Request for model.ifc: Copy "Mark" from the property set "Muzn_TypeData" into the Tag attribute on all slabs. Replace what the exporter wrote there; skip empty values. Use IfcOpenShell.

First a look at what the model holds.

```python
import ifcopenshell
import ifcopenshell.util.element

model = ifcopenshell.open("model.ifc")
print(model.schema)
slabs = model.by_type("IfcSlab")
print(len(slabs), "slabs")
for e in slabs[:8]:
    source = ifcopenshell.util.element.get_pset(e, "Muzn_TypeData", "Mark")
    target = e.Tag
    print(e.id(), repr(source), repr(target), sep=" | ")
```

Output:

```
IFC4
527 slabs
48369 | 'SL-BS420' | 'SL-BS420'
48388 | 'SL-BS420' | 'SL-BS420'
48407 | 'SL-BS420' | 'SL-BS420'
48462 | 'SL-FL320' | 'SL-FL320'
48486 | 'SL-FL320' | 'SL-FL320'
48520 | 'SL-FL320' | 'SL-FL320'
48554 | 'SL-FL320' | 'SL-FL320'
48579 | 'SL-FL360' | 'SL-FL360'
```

```python
import ifcopenshell
import ifcopenshell.util.element

model = ifcopenshell.open("model.ifc")

count = 0
for e in model.by_type("IfcSlab"):
    value = ifcopenshell.util.element.get_pset(e, "Muzn_TypeData", "Mark")
    current = e.Tag
    if not value or not value.strip() or current == value:
        continue
    e.Tag = value
    count += 1

print(count, "slabs updated")

model.write("model_updated.ifc")
```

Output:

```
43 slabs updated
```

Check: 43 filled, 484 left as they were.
